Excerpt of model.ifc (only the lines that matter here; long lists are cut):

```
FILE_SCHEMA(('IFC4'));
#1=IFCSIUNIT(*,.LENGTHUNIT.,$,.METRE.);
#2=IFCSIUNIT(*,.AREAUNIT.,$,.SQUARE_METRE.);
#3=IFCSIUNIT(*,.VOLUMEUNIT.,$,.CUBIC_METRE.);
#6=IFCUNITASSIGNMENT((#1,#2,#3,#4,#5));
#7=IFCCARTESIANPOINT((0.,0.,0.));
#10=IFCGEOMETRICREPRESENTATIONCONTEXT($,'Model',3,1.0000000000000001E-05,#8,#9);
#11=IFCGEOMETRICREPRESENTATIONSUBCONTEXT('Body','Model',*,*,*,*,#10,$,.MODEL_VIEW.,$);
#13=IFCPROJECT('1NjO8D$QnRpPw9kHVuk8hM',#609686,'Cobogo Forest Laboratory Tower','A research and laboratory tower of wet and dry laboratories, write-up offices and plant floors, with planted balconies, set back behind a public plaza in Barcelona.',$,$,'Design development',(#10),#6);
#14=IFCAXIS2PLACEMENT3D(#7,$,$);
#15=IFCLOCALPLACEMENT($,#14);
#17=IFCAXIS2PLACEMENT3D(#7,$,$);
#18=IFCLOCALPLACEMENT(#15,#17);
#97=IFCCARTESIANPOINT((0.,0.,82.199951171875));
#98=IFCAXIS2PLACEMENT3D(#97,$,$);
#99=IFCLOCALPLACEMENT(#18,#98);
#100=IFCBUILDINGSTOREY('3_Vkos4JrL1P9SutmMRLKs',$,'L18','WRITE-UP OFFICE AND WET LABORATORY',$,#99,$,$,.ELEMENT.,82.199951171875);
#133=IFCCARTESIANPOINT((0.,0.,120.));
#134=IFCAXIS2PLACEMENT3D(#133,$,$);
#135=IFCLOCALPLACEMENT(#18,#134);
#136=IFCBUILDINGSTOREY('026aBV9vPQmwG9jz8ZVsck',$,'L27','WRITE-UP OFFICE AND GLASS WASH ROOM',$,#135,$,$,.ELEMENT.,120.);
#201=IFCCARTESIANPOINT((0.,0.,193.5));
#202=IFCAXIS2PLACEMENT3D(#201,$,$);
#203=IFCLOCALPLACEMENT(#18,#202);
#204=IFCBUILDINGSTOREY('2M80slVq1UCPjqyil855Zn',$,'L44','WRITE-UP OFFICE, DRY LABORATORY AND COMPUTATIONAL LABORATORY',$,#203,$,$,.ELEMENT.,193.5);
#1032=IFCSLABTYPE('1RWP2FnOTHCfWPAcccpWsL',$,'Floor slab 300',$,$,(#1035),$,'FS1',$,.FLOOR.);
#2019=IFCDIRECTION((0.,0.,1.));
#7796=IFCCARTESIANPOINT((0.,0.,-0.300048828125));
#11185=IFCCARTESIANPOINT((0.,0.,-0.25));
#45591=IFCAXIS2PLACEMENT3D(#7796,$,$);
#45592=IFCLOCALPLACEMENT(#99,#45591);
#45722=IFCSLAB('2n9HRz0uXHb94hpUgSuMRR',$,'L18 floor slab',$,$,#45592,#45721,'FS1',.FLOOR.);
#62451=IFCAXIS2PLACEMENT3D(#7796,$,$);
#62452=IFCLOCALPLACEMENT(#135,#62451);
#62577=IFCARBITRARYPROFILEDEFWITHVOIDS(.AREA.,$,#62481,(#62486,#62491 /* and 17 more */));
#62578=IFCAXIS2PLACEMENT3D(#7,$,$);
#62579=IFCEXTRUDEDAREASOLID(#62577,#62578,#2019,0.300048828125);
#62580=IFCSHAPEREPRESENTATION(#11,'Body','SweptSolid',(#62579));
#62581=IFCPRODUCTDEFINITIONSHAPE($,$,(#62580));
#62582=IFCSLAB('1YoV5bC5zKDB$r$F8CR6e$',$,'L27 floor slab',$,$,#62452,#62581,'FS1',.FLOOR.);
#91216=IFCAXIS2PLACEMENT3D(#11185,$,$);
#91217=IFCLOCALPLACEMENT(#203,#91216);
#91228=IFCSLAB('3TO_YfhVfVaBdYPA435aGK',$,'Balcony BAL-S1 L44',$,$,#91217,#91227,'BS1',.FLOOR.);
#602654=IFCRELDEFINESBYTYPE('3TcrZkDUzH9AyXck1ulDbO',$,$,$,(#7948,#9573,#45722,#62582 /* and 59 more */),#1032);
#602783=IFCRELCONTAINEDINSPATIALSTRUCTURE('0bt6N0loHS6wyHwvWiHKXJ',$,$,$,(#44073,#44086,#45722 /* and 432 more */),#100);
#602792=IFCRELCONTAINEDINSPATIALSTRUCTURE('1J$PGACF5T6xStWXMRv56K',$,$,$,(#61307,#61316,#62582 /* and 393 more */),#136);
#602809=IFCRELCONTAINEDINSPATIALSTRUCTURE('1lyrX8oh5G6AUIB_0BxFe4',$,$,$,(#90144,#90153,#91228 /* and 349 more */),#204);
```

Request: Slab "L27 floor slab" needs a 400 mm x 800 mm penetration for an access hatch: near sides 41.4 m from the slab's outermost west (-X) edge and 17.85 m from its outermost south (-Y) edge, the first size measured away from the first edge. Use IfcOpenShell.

```python
import numpy as np
import ifcopenshell
import ifcopenshell.api.feature
import ifcopenshell.api.geometry
import ifcopenshell.api.root
import ifcopenshell.geom
import ifcopenshell.util.placement
import ifcopenshell.util.representation
import ifcopenshell.util.shape
import ifcopenshell.util.unit

model = ifcopenshell.open("model.ifc")
unit_scale = ifcopenshell.util.unit.calculate_unit_scale(model)
settings = ifcopenshell.geom.settings()


def volume(element):
    """Net volume in cubic metres, openings subtracted."""
    shape = ifcopenshell.geom.create_shape(settings, element)
    return ifcopenshell.util.shape.get_volume(shape.geometry)


slab = model.by_guid("1YoV5bC5zKDB$r$F8CR6e$")
before = volume(slab)

# Extent in the slab's own axes, in metres. The edges named are its -X and -Y sides.
slab_shape = ifcopenshell.geom.create_shape(settings, slab)
vertices = ifcopenshell.util.shape.get_vertices(slab_shape.geometry)
x_min, y_min, bottom = vertices.min(axis=0)
top = vertices[:, 2].max()

opening = ifcopenshell.api.root.create_entity(model, ifc_class="IfcOpeningElement", name="Access hatch opening", predefined_type="OPENING")
context = ifcopenshell.util.representation.get_context(model, "Model", "Body", "MODEL_VIEW")
width, depth = 0.4, 0.8
outline = [(0.0, 0.0), (width, 0.0), (width, depth), (0.0, depth), (0.0, 0.0)]
# Overshoot both faces by 50 mm so the cut is clean.
shape = ifcopenshell.api.geometry.add_slab_representation(
    model, context=context, depth=top - bottom + 0.1, polyline=outline
)
ifcopenshell.api.geometry.assign_representation(model, product=opening, representation=shape)

matrix = ifcopenshell.util.placement.get_local_placement(slab.ObjectPlacement)
matrix[:, 3] = matrix @ np.append(np.array([x_min + 41.4, y_min + 17.85, bottom - 0.05]) / unit_scale, 1.0)
ifcopenshell.api.geometry.edit_object_placement(model, product=opening, matrix=matrix, is_si=False)
ifcopenshell.api.feature.add_feature(model, feature=opening, element=slab)

after = volume(slab)

print(f"slab volume {before:.3f} -> {after:.3f} m3")

model.write("model-out.ifc")
```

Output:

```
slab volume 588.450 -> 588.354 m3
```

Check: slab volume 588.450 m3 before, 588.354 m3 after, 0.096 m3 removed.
